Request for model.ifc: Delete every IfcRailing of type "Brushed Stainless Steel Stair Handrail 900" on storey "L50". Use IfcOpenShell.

First a look at what the model holds.

```python
import ifcopenshell
import ifcopenshell.util.element

model = ifcopenshell.open("model.ifc")
print(model.schema)
storey = next(s for s in model.by_type("IfcBuildingStorey") if s.Name == "L50")
railings = [e for e in ifcopenshell.util.element.get_decomposition(storey) if e.is_a("IfcRailing")]
seen = {}
for e in railings:
    element_type = ifcopenshell.util.element.get_type(e)
    name = element_type.Name if element_type not in (None, e) else None
    seen[name] = seen.get(name, 0) + 1
for name, count in sorted(seen.items(), key=str):
    print(count, "x", name)
```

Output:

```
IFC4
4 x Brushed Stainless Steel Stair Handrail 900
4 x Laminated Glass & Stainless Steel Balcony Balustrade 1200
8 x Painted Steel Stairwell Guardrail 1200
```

```python
import ifcopenshell
import ifcopenshell.api.root
import ifcopenshell.util.element

model = ifcopenshell.open("model.ifc")

storey = next(s for s in model.by_type("IfcBuildingStorey") if s.Name == "L50")
railings = [e for e in ifcopenshell.util.element.get_decomposition(storey) if e.is_a("IfcRailing")]
targets = [e for e in railings if (t := ifcopenshell.util.element.get_type(e)) not in (None, e) and t.Name == "Brushed Stainless Steel Stair Handrail 900"]

for e in targets:
    ifcopenshell.api.root.remove_product(model, product=e)
print(len(targets), "removed")

model.write("model-out.ifc")
```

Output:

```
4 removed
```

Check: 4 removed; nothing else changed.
